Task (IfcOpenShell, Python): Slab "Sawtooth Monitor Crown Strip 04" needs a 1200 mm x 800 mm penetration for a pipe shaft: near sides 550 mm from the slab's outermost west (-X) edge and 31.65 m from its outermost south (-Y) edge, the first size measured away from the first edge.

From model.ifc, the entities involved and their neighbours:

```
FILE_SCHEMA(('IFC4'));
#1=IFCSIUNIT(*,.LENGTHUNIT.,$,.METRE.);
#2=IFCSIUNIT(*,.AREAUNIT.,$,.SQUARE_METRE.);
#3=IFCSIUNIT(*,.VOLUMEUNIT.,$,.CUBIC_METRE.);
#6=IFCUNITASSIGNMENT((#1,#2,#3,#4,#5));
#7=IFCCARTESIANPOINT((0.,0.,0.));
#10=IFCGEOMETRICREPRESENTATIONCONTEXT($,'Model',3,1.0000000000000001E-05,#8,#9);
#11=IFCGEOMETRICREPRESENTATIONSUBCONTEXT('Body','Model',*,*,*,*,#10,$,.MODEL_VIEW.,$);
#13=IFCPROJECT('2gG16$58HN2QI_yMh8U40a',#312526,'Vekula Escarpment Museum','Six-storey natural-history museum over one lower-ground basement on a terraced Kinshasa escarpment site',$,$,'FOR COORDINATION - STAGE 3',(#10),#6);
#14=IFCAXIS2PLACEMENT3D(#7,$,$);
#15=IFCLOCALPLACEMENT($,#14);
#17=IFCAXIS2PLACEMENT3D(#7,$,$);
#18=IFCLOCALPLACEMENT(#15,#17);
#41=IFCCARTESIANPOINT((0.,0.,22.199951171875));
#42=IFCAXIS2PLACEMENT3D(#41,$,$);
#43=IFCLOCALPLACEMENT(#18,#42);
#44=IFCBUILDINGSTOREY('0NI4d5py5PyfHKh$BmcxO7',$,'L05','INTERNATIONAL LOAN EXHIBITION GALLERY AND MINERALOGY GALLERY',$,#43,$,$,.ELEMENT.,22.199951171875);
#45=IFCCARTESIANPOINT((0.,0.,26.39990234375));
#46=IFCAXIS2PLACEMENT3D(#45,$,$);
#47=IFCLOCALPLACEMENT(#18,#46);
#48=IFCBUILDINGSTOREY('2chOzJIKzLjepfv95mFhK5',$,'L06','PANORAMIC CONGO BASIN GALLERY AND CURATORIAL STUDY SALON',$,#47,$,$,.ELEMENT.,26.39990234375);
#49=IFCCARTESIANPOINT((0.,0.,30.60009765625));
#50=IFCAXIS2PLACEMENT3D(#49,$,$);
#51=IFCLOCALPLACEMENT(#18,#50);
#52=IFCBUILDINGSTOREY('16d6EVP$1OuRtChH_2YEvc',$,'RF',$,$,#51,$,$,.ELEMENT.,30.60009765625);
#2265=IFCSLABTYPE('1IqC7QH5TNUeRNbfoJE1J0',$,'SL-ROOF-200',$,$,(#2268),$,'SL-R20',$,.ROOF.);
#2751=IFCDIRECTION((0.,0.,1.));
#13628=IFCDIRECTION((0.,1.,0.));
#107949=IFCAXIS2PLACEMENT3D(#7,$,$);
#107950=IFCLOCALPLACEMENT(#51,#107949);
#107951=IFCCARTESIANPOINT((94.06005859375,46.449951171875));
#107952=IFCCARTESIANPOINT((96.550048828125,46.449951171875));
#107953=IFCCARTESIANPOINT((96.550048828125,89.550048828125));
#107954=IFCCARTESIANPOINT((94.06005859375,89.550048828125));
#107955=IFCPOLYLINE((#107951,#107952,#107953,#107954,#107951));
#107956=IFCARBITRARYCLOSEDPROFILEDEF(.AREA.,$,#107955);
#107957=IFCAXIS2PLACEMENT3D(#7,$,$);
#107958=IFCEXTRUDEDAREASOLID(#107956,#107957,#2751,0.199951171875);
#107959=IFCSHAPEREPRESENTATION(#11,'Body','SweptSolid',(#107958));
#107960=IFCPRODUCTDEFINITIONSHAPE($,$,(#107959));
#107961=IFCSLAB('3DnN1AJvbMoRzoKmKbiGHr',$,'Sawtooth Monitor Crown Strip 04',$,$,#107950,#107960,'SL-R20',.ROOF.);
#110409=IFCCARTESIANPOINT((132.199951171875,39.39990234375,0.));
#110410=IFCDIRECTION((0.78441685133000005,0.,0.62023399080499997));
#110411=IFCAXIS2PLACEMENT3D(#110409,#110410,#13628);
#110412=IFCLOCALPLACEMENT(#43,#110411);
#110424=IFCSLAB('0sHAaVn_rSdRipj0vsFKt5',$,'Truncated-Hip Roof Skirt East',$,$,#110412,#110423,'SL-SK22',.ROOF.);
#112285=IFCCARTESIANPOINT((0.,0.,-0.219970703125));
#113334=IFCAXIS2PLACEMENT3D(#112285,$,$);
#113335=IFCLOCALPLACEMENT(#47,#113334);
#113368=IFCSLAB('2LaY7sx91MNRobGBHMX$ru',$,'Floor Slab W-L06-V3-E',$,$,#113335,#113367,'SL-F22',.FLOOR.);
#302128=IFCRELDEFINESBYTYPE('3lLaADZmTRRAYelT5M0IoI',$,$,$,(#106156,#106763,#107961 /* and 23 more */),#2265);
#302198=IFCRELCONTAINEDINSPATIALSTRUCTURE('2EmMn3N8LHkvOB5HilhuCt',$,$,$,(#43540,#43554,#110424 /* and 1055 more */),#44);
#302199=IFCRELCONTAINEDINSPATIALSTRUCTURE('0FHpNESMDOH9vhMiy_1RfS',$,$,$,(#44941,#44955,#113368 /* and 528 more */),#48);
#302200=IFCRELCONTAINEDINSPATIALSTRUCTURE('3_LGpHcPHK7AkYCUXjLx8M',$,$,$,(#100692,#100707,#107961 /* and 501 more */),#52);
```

```python
import numpy as np
import ifcopenshell
import ifcopenshell.api.feature
import ifcopenshell.api.geometry
import ifcopenshell.api.root
import ifcopenshell.geom
import ifcopenshell.util.placement
import ifcopenshell.util.representation
import ifcopenshell.util.shape
import ifcopenshell.util.unit

model = ifcopenshell.open("model.ifc")
unit_scale = ifcopenshell.util.unit.calculate_unit_scale(model)
settings = ifcopenshell.geom.settings()


def volume(element):
    """Net volume in cubic metres, openings subtracted."""
    shape = ifcopenshell.geom.create_shape(settings, element)
    return ifcopenshell.util.shape.get_volume(shape.geometry)


slab = model.by_guid("3DnN1AJvbMoRzoKmKbiGHr")
before = volume(slab)

# Extent in the slab's own axes, in metres. The edges named are its -X and -Y sides.
slab_shape = ifcopenshell.geom.create_shape(settings, slab)
vertices = ifcopenshell.util.shape.get_vertices(slab_shape.geometry)
x_min, y_min, bottom = vertices.min(axis=0)
top = vertices[:, 2].max()

opening = ifcopenshell.api.root.create_entity(model, ifc_class="IfcOpeningElement", name="Pipe shaft opening", predefined_type="OPENING")
context = ifcopenshell.util.representation.get_context(model, "Model", "Body", "MODEL_VIEW")
width, depth = 1.2, 0.8
outline = [(0.0, 0.0), (width, 0.0), (width, depth), (0.0, depth), (0.0, 0.0)]
# Overshoot both faces by 50 mm so the cut is clean.
shape = ifcopenshell.api.geometry.add_slab_representation(
    model, context=context, depth=top - bottom + 0.1, polyline=outline
)
ifcopenshell.api.geometry.assign_representation(model, product=opening, representation=shape)

matrix = ifcopenshell.util.placement.get_local_placement(slab.ObjectPlacement)
matrix[:, 3] = matrix @ np.append(np.array([x_min + 0.55, y_min + 31.65, bottom - 0.05]) / unit_scale, 1.0)
ifcopenshell.api.geometry.edit_object_placement(model, product=opening, matrix=matrix, is_si=False)
ifcopenshell.api.feature.add_feature(model, feature=opening, element=slab)

after = volume(slab)

print(f"slab volume {before:.3f} -> {after:.3f} m3")

model.write("model_updated.ifc")
```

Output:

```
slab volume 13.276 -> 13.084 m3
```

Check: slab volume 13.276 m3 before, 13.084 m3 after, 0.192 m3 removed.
